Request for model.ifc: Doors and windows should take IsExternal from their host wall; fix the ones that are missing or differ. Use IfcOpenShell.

First a look at what the model holds.

```python
import ifcopenshell
import ifcopenshell.util.element

model = ifcopenshell.open("model.ifc")
print(model.schema)
seen = {}
for e in model.by_type("IfcDoor") + model.by_type("IfcWindow"):
    if not e.FillsVoids:
        continue
    host = e.FillsVoids[0].RelatingOpeningElement.VoidsElements[0].RelatingBuildingElement
    own = ifcopenshell.util.element.get_pset(e, f"Pset_{e.is_a()[3:].removesuffix('StandardCase')}Common", "IsExternal")
    wall = ifcopenshell.util.element.get_pset(host, "Pset_WallCommon", "IsExternal")
    seen[e.is_a(), own, wall] = seen.get((e.is_a(), own, wall), 0) + 1
for (cls, own, wall), count in sorted(seen.items(), key=str):
    print(count, cls, "IsExternal:", own, "| host wall:", wall)
```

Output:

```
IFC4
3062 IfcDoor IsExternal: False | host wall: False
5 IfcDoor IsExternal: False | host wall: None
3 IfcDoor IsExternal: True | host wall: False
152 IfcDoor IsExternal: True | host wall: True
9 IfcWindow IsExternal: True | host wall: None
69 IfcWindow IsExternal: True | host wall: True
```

```python
import ifcopenshell
import ifcopenshell.api.pset
import ifcopenshell.util.element

model = ifcopenshell.open("model.ifc")

count = 0
for ifc_class, pset_name in (("IfcDoor", "Pset_DoorCommon"), ("IfcWindow", "Pset_WindowCommon")):
    for e in model.by_type(ifc_class):
        if not e.FillsVoids:
            continue
        host = e.FillsVoids[0].RelatingOpeningElement.VoidsElements[0].RelatingBuildingElement
        external = ifcopenshell.util.element.get_pset(host, "Pset_WallCommon", "IsExternal")
        if external is None or ifcopenshell.util.element.get_pset(e, pset_name, "IsExternal") == external:
            continue
        found = ifcopenshell.util.element.get_pset(e, pset_name, should_inherit=False)
        if found:
            pset = model.by_id(found["id"])
            if len(ifcopenshell.util.element.get_elements_by_pset(pset)) > 1:
                pset = ifcopenshell.api.pset.unshare_pset(model, products=[e], pset=pset)[0]
        else:
            pset = ifcopenshell.api.pset.add_pset(model, product=e, name=pset_name)
        ifcopenshell.api.pset.edit_pset(model, pset=pset, properties={"IsExternal": external})
        count += 1

print(count, "updated")

model.write("model_edited.ifc")
```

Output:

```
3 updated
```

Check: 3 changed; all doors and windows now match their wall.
